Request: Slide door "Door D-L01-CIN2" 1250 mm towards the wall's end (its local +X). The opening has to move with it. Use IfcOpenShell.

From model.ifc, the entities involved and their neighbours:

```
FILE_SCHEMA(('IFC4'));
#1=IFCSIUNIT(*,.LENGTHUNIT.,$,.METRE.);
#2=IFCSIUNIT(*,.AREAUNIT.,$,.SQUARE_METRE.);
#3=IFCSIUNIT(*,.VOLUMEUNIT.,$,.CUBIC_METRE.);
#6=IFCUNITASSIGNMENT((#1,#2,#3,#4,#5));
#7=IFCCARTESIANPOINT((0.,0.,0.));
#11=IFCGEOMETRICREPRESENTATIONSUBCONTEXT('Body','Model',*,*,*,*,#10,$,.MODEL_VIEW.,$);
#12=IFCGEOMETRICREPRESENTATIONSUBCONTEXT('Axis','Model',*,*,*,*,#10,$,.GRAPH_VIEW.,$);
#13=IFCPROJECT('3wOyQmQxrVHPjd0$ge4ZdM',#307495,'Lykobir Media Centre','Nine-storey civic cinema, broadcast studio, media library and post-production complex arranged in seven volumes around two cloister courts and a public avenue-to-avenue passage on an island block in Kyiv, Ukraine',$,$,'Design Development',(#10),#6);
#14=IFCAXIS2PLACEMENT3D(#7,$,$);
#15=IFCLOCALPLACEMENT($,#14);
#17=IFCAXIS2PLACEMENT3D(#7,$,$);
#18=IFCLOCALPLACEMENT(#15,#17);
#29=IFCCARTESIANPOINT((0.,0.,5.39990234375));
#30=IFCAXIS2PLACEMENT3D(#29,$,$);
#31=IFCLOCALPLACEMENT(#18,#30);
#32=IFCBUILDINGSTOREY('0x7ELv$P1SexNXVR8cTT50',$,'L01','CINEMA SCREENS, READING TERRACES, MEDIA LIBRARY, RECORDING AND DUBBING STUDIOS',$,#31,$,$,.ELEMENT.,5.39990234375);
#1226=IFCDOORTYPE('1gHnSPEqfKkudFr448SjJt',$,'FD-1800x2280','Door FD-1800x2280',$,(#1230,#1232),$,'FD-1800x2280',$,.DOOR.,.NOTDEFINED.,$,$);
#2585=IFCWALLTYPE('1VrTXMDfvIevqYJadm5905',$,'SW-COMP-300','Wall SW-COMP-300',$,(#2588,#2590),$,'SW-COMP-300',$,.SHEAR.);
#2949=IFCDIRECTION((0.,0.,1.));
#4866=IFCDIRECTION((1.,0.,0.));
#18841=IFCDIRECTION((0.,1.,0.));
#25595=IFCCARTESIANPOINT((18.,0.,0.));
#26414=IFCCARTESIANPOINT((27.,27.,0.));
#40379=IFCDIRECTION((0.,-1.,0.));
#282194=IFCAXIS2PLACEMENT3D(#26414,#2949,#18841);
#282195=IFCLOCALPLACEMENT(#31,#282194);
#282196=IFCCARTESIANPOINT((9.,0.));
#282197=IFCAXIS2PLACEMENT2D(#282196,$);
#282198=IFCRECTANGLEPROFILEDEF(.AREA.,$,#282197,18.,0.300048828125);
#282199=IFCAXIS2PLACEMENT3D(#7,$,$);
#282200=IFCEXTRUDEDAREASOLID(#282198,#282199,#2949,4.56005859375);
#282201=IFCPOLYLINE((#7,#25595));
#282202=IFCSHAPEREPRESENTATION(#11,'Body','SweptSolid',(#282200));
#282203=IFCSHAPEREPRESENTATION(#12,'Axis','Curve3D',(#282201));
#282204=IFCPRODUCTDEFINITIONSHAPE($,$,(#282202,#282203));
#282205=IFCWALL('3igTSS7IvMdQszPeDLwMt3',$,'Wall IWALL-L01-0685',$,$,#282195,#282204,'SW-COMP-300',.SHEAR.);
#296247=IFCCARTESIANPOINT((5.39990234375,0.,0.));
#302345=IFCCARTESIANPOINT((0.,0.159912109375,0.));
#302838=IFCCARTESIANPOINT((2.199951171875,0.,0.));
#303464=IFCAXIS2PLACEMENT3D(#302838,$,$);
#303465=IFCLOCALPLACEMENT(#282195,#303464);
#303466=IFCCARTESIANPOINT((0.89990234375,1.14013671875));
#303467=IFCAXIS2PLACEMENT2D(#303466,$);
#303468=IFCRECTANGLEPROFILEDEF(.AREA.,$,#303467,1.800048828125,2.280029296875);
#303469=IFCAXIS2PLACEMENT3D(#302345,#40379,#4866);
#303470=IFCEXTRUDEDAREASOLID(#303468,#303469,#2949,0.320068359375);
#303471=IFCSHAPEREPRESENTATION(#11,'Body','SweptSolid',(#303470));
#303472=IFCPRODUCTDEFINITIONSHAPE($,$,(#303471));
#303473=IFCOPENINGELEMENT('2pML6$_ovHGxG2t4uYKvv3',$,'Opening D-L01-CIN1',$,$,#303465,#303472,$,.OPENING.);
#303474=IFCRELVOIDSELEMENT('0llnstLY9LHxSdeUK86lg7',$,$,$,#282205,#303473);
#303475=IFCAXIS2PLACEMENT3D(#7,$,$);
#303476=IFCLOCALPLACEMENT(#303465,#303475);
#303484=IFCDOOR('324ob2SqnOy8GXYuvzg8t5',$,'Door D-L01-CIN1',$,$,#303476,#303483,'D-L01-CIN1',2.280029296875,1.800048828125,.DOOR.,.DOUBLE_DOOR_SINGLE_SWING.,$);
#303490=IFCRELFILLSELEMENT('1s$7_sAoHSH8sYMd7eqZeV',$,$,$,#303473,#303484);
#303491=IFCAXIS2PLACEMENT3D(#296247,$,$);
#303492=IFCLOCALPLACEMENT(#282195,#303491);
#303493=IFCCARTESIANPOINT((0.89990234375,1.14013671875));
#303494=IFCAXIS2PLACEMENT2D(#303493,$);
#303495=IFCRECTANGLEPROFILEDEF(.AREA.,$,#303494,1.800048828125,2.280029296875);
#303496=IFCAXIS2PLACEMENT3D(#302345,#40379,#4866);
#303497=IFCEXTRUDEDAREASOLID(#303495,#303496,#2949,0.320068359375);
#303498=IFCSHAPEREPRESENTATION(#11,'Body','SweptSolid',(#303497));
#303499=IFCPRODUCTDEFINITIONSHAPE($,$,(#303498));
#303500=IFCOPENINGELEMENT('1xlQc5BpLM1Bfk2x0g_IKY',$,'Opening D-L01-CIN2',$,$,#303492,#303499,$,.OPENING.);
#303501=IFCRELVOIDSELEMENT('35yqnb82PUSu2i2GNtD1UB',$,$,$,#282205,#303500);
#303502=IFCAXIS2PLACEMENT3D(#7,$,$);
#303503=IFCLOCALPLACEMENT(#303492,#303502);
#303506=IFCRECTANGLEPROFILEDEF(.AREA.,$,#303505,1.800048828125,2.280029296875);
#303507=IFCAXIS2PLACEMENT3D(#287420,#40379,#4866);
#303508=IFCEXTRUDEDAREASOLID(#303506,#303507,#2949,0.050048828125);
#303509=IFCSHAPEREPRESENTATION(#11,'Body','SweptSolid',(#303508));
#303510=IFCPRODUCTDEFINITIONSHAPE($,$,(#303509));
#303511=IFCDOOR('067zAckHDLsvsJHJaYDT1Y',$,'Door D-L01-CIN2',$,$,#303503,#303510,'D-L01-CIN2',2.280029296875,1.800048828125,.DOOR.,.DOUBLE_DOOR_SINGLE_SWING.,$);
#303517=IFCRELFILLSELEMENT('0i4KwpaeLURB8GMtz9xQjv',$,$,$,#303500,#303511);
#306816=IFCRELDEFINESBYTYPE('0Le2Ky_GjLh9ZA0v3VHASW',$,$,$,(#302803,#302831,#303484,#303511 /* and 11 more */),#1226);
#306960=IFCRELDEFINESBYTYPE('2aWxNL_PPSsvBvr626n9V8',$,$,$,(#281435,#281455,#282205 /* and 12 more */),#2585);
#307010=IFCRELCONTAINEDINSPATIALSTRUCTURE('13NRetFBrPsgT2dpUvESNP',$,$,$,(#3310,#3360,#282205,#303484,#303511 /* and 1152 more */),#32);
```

```python
import ifcopenshell
import ifcopenshell.api.geometry
import ifcopenshell.util.placement
import ifcopenshell.util.unit

model = ifcopenshell.open("model.ifc")
unit_scale = ifcopenshell.util.unit.calculate_unit_scale(model)

door = model.by_guid("067zAckHDLsvsJHJaYDT1Y")
opening = door.FillsVoids[0].RelatingOpeningElement
wall = opening.VoidsElements[0].RelatingBuildingElement

wall_matrix = ifcopenshell.util.placement.get_local_placement(wall.ObjectPlacement)
shift = wall_matrix[:3, 0] * 1.25 / unit_scale
before = ifcopenshell.util.placement.get_local_placement(door.ObjectPlacement)[:3, 3].copy()

# The door is placed relative to its opening, so it follows when the opening moves.
matrix = ifcopenshell.util.placement.get_local_placement(opening.ObjectPlacement)
matrix[:3, 3] += shift
ifcopenshell.api.geometry.edit_object_placement(
    model, product=opening, matrix=matrix, is_si=False, should_transform_children=True
)

after = ifcopenshell.util.placement.get_local_placement(door.ObjectPlacement)[:3, 3]
print("door moved by", (after - before).round(3) + 0.0)

model.write("model_updated.ifc")
```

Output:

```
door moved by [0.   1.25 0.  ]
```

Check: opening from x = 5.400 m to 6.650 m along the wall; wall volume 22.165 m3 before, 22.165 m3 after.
